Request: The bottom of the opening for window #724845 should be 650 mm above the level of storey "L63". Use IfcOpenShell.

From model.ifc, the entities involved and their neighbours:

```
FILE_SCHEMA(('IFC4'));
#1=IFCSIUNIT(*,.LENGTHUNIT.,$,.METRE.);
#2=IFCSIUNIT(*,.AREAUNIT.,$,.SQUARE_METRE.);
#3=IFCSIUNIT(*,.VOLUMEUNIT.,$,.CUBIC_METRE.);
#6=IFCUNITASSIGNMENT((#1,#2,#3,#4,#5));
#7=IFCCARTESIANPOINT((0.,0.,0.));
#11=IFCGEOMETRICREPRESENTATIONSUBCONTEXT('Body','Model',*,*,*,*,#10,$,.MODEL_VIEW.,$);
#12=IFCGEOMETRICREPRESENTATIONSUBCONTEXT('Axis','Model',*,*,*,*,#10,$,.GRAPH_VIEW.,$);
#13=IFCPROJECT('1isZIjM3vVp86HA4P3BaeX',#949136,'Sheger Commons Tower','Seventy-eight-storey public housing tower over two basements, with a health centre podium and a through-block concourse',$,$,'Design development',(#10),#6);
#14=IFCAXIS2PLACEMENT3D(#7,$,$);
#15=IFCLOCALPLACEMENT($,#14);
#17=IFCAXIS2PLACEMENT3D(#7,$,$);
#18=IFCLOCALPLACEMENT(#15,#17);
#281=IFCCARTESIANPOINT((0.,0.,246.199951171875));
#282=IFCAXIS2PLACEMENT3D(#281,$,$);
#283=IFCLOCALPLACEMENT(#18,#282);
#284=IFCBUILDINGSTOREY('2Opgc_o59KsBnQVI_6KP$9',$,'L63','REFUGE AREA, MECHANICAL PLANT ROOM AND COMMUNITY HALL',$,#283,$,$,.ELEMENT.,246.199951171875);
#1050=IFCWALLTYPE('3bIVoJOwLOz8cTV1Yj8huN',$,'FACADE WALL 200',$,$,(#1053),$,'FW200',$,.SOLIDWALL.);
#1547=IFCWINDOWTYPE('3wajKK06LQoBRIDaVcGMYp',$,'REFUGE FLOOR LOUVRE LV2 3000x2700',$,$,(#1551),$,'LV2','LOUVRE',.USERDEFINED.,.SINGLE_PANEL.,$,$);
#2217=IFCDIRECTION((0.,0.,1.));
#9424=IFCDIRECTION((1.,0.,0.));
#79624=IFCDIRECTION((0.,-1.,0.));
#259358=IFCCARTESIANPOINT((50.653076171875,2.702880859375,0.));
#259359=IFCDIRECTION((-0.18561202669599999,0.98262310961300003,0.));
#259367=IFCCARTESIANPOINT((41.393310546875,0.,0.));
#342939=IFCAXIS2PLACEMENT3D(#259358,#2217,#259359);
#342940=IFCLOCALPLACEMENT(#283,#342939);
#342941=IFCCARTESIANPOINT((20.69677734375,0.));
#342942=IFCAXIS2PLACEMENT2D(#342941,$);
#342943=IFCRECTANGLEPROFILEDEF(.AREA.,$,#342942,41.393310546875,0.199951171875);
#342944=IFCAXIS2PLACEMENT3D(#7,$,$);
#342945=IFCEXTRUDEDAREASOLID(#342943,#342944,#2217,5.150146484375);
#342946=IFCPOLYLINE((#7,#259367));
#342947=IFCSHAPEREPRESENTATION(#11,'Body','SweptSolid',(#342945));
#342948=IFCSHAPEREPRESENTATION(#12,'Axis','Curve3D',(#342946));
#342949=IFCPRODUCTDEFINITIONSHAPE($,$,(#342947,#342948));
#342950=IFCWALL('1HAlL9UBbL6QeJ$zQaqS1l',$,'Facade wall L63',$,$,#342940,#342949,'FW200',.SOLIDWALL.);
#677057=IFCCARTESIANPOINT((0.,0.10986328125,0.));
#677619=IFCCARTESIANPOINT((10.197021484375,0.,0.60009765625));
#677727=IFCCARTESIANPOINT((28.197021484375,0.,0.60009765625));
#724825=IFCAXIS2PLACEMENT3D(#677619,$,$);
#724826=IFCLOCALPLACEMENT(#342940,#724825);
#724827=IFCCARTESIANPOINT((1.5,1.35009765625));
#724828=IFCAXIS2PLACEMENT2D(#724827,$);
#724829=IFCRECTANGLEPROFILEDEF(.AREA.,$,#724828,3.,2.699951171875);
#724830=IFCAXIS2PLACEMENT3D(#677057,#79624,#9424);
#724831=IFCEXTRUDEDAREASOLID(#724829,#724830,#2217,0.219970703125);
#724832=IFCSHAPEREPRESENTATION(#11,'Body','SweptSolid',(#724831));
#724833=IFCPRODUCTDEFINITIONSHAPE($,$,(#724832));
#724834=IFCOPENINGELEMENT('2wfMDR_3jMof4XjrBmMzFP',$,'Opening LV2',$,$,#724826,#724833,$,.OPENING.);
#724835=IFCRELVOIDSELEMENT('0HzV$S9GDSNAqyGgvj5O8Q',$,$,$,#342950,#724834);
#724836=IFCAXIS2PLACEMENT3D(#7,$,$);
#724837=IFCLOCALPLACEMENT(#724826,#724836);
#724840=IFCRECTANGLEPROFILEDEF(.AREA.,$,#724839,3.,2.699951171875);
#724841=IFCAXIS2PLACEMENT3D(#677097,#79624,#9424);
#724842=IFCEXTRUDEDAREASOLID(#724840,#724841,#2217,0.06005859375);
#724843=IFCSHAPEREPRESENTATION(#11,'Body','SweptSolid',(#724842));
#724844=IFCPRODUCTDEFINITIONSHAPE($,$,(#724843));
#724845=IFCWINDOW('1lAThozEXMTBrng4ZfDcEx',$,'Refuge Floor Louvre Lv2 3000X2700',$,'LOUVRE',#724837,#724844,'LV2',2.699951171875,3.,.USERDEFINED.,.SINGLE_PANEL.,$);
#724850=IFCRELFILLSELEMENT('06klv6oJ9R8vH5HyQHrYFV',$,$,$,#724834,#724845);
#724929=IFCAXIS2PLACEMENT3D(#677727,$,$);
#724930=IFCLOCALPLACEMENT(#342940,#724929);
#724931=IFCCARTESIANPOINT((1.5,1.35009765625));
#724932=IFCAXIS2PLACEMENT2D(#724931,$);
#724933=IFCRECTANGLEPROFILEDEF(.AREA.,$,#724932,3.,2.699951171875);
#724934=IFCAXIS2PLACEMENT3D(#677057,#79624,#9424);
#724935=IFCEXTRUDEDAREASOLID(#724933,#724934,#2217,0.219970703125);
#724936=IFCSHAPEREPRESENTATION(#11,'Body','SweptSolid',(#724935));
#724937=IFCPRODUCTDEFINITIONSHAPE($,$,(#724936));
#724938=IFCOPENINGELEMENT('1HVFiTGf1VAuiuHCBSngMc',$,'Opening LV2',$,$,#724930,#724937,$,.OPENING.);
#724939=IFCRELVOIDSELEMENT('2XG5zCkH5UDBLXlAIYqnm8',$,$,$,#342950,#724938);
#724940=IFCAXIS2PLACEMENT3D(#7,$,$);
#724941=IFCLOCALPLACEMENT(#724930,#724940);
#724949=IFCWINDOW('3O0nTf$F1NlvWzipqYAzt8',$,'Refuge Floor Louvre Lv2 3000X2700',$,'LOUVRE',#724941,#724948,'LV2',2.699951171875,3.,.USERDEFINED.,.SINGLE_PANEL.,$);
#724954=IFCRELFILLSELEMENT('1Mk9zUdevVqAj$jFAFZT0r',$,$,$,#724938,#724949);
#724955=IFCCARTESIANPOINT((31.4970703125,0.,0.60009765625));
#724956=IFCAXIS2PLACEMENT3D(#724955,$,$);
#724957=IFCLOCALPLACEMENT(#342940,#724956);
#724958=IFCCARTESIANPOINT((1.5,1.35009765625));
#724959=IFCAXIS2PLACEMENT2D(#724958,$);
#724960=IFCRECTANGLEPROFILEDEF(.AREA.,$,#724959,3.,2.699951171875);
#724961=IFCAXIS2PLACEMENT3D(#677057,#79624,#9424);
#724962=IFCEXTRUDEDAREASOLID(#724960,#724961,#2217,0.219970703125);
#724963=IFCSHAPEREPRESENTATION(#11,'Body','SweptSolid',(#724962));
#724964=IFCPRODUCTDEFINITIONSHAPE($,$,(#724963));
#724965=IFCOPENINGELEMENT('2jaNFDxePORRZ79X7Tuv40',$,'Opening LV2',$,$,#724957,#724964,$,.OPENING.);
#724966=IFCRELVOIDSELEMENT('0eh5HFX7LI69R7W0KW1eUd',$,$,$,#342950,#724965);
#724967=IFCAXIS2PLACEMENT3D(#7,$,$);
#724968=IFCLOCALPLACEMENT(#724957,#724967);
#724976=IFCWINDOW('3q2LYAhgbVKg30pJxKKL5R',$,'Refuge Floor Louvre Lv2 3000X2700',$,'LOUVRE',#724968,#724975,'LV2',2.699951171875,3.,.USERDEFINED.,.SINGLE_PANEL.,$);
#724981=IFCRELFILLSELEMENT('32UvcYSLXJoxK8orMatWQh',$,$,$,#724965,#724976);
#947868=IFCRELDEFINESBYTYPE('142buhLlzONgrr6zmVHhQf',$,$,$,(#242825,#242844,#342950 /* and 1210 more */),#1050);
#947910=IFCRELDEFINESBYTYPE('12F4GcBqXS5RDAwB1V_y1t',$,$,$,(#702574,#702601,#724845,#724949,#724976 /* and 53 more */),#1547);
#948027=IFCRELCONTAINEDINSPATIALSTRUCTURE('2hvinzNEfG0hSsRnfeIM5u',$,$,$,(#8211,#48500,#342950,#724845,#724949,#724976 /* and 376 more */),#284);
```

```python
import numpy as np
import ifcopenshell
import ifcopenshell.api.geometry
import ifcopenshell.geom
import ifcopenshell.util.element
import ifcopenshell.util.placement
import ifcopenshell.util.shape
import ifcopenshell.util.unit

model = ifcopenshell.open("model.ifc")
unit_scale = ifcopenshell.util.unit.calculate_unit_scale(model)

window = model.by_guid("1lAThozEXMTBrng4ZfDcEx")
opening = window.FillsVoids[0].RelatingOpeningElement
storey = ifcopenshell.util.element.get_container(window, ifc_class="IfcBuildingStorey")
level = ifcopenshell.util.placement.get_local_placement(storey.ObjectPlacement)[2, 3]

# The opening's origin need not be at the sill, so measure its lowest point.
shape = ifcopenshell.geom.create_shape(ifcopenshell.geom.settings(), opening)
bottom = ifcopenshell.util.shape.get_shape_bottom_elevation(shape, shape.geometry) / unit_scale
dz = level + 0.65 / unit_scale - bottom

shift = np.array([0.0, 0.0, dz])
# The window is placed relative to its opening, so it follows when the opening moves.
matrix = ifcopenshell.util.placement.get_local_placement(opening.ObjectPlacement)
matrix[:3, 3] += shift
ifcopenshell.api.geometry.edit_object_placement(
    model, product=opening, matrix=matrix, is_si=False, should_transform_children=True
)

print(f"moved by {dz * unit_scale:+.3f} m")

model.write("model_updated.ifc")
```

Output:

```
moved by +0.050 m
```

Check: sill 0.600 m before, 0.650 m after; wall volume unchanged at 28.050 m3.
